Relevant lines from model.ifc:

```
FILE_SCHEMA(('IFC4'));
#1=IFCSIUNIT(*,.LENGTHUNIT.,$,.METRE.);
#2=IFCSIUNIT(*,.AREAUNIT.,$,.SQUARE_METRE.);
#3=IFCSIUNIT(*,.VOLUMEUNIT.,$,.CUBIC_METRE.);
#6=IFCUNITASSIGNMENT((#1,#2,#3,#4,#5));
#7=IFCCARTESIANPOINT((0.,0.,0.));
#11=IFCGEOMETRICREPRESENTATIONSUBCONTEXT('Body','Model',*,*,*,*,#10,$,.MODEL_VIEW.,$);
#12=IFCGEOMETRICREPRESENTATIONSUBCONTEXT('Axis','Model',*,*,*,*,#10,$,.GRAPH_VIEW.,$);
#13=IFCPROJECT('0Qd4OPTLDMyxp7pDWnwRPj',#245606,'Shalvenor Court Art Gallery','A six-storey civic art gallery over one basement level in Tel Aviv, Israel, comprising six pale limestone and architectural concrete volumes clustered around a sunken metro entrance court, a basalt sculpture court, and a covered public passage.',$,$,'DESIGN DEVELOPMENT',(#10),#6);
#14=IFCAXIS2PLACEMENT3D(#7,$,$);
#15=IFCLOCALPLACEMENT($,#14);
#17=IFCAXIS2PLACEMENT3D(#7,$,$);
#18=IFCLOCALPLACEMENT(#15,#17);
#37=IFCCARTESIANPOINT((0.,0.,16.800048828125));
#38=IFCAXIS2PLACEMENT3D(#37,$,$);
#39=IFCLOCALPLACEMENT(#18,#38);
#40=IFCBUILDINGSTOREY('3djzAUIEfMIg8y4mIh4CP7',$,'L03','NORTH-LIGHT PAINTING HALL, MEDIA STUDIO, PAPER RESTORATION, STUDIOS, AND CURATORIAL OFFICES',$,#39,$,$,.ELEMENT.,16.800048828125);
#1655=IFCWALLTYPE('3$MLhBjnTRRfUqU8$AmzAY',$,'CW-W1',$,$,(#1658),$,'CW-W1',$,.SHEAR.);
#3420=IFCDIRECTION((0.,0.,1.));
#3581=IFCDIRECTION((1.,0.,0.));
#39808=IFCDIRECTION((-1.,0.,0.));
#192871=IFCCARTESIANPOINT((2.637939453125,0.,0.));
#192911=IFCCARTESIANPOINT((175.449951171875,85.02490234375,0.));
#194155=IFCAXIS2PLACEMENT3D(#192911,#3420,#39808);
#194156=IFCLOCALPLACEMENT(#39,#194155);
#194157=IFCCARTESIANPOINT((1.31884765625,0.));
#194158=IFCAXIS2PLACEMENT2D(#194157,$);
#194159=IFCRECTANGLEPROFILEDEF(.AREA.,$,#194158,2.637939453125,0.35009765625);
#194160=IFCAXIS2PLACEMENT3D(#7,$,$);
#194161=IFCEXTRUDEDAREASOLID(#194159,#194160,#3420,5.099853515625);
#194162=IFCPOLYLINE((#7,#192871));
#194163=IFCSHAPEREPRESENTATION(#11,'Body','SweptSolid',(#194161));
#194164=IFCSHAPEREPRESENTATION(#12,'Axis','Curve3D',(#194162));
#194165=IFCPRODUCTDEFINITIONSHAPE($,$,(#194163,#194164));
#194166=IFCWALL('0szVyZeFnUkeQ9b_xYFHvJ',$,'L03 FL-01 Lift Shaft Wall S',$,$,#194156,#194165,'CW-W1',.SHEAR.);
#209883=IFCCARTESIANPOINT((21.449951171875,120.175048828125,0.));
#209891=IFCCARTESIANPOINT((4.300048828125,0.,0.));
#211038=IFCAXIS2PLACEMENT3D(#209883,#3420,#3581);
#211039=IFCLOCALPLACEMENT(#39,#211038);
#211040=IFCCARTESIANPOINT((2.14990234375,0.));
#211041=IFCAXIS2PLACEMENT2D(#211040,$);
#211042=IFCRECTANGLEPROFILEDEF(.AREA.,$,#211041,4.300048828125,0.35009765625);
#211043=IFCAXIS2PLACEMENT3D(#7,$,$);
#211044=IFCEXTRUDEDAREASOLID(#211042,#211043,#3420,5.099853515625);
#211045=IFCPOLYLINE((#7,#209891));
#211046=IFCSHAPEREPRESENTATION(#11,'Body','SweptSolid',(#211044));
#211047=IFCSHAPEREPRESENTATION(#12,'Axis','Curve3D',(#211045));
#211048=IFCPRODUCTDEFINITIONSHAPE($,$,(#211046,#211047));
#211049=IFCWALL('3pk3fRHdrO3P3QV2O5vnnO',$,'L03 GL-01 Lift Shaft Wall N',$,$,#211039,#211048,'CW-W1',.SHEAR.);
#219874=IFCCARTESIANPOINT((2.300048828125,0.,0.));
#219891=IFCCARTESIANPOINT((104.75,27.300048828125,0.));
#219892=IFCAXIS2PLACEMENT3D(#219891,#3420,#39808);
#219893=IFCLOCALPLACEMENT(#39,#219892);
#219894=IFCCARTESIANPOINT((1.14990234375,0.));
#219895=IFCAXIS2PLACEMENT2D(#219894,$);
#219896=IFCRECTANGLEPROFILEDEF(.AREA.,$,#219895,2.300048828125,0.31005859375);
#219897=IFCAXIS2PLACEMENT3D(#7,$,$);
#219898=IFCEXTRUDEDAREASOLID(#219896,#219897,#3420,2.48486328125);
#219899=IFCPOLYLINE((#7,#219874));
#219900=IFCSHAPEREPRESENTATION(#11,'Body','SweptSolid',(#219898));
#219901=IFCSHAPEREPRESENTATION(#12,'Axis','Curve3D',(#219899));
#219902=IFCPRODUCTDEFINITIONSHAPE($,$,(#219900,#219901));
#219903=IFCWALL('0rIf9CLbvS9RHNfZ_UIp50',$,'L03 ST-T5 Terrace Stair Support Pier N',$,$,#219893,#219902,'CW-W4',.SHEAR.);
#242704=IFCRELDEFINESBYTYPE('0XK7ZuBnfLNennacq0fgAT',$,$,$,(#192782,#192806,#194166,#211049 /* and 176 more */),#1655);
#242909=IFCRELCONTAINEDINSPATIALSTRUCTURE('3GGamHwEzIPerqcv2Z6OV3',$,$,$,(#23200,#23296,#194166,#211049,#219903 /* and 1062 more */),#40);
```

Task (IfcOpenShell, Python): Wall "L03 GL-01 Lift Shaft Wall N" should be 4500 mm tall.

```python
import ifcopenshell
import ifcopenshell.geom
import ifcopenshell.util.representation
import ifcopenshell.util.shape
import ifcopenshell.util.unit

model = ifcopenshell.open("model.ifc")
unit_scale = ifcopenshell.util.unit.calculate_unit_scale(model)
settings = ifcopenshell.geom.settings()


def volume(element):
    """Net volume in cubic metres, openings subtracted."""
    shape = ifcopenshell.geom.create_shape(settings, element)
    return ifcopenshell.util.shape.get_volume(shape.geometry)


wall = model.by_id(211049)
before = volume(wall)

body = ifcopenshell.util.representation.get_representation(wall, "Model", "Body")
solid = body.Items[0]
old_height = solid.Depth
solid.Depth = 4.5 / unit_scale
after = volume(wall)

print(f"height {old_height:g} -> {solid.Depth:g}, volume {before:.3f} -> {after:.3f} m3")

model.write("model_v2.ifc")
```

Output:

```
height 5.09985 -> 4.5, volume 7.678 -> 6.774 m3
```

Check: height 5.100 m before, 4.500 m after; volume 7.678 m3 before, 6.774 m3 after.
